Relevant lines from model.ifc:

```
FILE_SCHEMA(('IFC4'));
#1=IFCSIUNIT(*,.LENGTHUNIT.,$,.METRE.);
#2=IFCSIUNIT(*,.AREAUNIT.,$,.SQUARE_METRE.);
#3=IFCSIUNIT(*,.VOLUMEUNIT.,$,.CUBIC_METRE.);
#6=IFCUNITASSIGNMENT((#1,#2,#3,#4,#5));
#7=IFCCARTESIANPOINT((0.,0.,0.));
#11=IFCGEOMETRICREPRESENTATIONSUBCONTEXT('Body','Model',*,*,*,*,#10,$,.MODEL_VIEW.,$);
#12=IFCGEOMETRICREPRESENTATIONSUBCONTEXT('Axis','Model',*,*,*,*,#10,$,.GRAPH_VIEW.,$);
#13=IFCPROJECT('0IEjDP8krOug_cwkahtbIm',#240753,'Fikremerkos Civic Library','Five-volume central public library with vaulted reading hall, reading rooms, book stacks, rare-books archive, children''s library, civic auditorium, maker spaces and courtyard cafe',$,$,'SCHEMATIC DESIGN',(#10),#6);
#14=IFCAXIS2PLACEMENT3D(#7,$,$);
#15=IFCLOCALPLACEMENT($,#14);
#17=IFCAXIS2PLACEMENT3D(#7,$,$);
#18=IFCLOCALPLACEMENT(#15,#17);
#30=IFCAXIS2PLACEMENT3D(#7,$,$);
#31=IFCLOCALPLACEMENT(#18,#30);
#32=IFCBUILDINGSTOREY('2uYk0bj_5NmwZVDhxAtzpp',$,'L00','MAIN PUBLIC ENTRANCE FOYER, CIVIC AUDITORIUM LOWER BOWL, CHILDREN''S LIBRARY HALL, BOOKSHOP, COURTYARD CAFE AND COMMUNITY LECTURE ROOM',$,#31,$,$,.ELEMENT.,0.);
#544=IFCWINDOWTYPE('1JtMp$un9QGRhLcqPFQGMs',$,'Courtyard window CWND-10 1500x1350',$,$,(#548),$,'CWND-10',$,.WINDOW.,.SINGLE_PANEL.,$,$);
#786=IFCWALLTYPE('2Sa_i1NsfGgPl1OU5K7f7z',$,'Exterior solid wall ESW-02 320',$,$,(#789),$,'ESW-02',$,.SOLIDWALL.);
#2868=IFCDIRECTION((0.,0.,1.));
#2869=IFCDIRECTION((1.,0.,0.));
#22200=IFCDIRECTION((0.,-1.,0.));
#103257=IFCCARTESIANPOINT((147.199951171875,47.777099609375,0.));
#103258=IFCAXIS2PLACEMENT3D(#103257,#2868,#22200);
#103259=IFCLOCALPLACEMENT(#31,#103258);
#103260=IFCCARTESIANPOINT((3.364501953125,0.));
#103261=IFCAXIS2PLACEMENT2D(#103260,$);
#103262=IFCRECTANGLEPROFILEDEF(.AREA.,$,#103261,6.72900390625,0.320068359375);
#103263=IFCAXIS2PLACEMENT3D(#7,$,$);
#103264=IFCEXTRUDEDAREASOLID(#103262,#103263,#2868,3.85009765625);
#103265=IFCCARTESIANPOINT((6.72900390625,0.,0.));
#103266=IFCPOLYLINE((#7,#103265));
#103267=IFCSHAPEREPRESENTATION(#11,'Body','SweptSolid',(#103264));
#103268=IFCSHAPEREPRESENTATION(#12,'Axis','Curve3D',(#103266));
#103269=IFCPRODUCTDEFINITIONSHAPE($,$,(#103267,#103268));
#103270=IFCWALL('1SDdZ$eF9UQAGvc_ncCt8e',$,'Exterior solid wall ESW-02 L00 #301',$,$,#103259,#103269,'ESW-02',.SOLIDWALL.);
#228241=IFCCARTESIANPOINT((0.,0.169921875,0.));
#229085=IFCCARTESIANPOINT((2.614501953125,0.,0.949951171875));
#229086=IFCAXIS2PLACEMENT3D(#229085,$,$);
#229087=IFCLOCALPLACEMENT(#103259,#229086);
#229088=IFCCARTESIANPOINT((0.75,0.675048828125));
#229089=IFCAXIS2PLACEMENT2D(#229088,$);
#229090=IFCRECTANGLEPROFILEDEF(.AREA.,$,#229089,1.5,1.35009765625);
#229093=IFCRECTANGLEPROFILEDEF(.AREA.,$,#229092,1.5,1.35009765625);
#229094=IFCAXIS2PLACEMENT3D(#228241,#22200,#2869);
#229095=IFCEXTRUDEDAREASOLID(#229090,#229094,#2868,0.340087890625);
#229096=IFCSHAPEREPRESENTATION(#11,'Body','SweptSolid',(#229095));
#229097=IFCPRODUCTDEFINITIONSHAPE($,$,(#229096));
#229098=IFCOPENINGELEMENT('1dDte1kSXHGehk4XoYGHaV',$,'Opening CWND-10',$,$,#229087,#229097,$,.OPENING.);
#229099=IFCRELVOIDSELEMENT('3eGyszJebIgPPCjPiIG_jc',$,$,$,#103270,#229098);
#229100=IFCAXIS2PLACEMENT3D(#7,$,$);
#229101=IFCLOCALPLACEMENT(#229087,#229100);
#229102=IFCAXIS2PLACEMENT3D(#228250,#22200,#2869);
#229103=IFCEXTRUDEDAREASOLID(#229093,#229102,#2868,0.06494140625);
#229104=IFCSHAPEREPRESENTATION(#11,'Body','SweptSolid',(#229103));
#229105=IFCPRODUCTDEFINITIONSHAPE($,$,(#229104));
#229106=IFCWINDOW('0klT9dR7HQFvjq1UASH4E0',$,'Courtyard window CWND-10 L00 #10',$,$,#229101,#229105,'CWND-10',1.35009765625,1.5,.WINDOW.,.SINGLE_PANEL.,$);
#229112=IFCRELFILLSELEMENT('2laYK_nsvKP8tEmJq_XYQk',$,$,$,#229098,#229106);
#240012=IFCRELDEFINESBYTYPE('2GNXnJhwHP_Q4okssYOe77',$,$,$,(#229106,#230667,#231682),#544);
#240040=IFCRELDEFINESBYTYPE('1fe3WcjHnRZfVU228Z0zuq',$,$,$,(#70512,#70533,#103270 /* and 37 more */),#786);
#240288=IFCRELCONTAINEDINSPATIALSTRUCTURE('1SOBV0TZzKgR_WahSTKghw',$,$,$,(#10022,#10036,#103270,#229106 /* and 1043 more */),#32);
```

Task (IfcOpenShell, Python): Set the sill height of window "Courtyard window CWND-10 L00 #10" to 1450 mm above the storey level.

```python
import numpy as np
import ifcopenshell
import ifcopenshell.api.geometry
import ifcopenshell.geom
import ifcopenshell.util.element
import ifcopenshell.util.placement
import ifcopenshell.util.shape
import ifcopenshell.util.unit

model = ifcopenshell.open("model.ifc")
unit_scale = ifcopenshell.util.unit.calculate_unit_scale(model)

window = model.by_guid("0klT9dR7HQFvjq1UASH4E0")
opening = window.FillsVoids[0].RelatingOpeningElement
storey = ifcopenshell.util.element.get_container(window, ifc_class="IfcBuildingStorey")
level = ifcopenshell.util.placement.get_local_placement(storey.ObjectPlacement)[2, 3]

# The opening's origin need not be at the sill, so measure its lowest point.
shape = ifcopenshell.geom.create_shape(ifcopenshell.geom.settings(), opening)
bottom = ifcopenshell.util.shape.get_shape_bottom_elevation(shape, shape.geometry) / unit_scale
dz = level + 1.45 - bottom

shift = np.array([0.0, 0.0, dz])
# The window is placed relative to its opening, so it follows when the opening moves.
matrix = ifcopenshell.util.placement.get_local_placement(opening.ObjectPlacement)
matrix[:3, 3] += shift
ifcopenshell.api.geometry.edit_object_placement(
    model, product=opening, matrix=matrix, is_si=False, should_transform_children=True
)

print(f"moved by {dz * unit_scale:+.3f} m")

model.write("model-out.ifc")
```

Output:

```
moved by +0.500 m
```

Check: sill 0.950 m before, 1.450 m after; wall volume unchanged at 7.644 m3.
